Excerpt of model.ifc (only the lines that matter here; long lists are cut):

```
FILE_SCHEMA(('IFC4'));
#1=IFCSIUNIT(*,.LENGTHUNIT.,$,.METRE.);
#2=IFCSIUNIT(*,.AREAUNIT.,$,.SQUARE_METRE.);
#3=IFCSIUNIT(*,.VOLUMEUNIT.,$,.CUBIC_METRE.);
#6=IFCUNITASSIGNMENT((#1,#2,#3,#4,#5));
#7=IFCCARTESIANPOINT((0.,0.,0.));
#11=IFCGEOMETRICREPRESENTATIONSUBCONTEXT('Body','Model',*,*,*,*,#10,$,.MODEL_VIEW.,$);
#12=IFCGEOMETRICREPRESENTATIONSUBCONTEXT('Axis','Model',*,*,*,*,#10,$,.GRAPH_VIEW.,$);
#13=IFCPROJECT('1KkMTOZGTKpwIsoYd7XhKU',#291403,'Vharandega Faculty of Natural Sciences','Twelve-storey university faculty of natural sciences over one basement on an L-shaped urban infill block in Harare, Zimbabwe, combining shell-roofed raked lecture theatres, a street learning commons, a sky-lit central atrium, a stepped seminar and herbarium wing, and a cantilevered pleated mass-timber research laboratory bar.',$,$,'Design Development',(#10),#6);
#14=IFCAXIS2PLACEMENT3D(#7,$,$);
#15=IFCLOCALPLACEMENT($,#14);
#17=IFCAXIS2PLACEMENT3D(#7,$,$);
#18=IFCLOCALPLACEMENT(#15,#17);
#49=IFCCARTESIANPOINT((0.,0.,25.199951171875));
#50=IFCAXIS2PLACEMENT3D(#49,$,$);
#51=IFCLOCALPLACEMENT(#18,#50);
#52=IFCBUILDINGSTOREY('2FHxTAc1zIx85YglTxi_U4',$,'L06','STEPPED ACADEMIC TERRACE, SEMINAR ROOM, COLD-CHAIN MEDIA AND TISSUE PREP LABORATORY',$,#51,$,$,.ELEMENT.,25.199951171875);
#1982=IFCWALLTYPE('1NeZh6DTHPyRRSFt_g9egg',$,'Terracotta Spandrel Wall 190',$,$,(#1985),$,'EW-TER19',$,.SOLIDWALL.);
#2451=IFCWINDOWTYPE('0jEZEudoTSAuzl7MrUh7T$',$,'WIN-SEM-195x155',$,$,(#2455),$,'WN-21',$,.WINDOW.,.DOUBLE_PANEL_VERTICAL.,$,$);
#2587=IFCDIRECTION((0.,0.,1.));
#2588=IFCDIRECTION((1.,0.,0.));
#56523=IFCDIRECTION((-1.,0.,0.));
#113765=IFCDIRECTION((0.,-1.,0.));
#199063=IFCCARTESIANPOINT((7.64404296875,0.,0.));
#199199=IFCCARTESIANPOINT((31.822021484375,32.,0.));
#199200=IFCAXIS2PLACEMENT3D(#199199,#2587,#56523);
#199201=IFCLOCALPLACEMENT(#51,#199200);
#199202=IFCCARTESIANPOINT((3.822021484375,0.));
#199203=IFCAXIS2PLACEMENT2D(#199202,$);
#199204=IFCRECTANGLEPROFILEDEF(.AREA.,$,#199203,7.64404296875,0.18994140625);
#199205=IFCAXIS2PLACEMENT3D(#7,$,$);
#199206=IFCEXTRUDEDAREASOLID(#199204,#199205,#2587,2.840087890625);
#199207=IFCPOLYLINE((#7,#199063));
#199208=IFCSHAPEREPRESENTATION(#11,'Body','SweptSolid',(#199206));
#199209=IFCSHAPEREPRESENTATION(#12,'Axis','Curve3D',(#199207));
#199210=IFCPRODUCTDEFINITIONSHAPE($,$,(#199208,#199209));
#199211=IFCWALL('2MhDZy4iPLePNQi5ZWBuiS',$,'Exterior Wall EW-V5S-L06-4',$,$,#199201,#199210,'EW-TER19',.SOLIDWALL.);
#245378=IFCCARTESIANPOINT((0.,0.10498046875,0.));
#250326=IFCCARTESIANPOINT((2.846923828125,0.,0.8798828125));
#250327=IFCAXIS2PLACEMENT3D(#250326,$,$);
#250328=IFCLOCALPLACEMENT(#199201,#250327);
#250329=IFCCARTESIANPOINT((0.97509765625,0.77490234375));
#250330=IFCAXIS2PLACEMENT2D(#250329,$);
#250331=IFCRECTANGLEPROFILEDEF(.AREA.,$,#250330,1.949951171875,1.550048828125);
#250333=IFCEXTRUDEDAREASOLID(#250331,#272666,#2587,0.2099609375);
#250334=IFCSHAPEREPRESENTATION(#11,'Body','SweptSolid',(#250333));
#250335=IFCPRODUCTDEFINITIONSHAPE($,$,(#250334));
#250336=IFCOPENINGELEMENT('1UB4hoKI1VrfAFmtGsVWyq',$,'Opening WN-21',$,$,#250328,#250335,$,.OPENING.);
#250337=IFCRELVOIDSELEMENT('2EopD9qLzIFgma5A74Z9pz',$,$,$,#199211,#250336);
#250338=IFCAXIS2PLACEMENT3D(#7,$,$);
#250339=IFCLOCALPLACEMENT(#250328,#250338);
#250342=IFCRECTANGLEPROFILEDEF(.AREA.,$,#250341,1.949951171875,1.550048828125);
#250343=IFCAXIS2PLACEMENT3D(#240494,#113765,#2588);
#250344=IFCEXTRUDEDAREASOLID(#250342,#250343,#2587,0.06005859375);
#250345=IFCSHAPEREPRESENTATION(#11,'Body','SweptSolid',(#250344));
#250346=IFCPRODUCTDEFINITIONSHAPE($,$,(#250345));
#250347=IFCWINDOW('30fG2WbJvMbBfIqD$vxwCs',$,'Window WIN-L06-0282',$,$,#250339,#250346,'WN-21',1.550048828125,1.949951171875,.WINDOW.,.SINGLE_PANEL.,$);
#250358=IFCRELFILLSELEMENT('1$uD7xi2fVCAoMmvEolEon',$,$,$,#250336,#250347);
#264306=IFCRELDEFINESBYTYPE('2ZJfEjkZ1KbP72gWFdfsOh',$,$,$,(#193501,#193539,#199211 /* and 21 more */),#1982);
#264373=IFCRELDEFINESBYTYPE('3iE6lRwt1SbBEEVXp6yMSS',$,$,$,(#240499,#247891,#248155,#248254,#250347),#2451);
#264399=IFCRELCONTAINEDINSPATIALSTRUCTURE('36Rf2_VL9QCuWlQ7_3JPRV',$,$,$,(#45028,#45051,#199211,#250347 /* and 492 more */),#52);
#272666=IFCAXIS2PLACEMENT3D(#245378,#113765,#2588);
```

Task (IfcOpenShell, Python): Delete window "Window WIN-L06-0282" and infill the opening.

```python
import ifcopenshell
import ifcopenshell.api.feature
import ifcopenshell.api.root
import ifcopenshell.geom
import ifcopenshell.util.shape

model = ifcopenshell.open("model.ifc")
settings = ifcopenshell.geom.settings()


def volume(element):
    """Net volume in cubic metres, openings subtracted."""
    shape = ifcopenshell.geom.create_shape(settings, element)
    return ifcopenshell.util.shape.get_volume(shape.geometry)


window = model.by_guid("30fG2WbJvMbBfIqD$vxwCs")
opening = window.FillsVoids[0].RelatingOpeningElement
wall = opening.VoidsElements[0].RelatingBuildingElement
before = volume(wall)

ifcopenshell.api.root.remove_product(model, product=window)
ifcopenshell.api.feature.remove_feature(model, feature=opening)

after = volume(wall)

print(f"wall volume {before:.3f} -> {after:.3f} m3")

model.write("model_rev.ifc")
```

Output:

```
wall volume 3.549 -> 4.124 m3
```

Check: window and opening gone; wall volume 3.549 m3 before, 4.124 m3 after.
